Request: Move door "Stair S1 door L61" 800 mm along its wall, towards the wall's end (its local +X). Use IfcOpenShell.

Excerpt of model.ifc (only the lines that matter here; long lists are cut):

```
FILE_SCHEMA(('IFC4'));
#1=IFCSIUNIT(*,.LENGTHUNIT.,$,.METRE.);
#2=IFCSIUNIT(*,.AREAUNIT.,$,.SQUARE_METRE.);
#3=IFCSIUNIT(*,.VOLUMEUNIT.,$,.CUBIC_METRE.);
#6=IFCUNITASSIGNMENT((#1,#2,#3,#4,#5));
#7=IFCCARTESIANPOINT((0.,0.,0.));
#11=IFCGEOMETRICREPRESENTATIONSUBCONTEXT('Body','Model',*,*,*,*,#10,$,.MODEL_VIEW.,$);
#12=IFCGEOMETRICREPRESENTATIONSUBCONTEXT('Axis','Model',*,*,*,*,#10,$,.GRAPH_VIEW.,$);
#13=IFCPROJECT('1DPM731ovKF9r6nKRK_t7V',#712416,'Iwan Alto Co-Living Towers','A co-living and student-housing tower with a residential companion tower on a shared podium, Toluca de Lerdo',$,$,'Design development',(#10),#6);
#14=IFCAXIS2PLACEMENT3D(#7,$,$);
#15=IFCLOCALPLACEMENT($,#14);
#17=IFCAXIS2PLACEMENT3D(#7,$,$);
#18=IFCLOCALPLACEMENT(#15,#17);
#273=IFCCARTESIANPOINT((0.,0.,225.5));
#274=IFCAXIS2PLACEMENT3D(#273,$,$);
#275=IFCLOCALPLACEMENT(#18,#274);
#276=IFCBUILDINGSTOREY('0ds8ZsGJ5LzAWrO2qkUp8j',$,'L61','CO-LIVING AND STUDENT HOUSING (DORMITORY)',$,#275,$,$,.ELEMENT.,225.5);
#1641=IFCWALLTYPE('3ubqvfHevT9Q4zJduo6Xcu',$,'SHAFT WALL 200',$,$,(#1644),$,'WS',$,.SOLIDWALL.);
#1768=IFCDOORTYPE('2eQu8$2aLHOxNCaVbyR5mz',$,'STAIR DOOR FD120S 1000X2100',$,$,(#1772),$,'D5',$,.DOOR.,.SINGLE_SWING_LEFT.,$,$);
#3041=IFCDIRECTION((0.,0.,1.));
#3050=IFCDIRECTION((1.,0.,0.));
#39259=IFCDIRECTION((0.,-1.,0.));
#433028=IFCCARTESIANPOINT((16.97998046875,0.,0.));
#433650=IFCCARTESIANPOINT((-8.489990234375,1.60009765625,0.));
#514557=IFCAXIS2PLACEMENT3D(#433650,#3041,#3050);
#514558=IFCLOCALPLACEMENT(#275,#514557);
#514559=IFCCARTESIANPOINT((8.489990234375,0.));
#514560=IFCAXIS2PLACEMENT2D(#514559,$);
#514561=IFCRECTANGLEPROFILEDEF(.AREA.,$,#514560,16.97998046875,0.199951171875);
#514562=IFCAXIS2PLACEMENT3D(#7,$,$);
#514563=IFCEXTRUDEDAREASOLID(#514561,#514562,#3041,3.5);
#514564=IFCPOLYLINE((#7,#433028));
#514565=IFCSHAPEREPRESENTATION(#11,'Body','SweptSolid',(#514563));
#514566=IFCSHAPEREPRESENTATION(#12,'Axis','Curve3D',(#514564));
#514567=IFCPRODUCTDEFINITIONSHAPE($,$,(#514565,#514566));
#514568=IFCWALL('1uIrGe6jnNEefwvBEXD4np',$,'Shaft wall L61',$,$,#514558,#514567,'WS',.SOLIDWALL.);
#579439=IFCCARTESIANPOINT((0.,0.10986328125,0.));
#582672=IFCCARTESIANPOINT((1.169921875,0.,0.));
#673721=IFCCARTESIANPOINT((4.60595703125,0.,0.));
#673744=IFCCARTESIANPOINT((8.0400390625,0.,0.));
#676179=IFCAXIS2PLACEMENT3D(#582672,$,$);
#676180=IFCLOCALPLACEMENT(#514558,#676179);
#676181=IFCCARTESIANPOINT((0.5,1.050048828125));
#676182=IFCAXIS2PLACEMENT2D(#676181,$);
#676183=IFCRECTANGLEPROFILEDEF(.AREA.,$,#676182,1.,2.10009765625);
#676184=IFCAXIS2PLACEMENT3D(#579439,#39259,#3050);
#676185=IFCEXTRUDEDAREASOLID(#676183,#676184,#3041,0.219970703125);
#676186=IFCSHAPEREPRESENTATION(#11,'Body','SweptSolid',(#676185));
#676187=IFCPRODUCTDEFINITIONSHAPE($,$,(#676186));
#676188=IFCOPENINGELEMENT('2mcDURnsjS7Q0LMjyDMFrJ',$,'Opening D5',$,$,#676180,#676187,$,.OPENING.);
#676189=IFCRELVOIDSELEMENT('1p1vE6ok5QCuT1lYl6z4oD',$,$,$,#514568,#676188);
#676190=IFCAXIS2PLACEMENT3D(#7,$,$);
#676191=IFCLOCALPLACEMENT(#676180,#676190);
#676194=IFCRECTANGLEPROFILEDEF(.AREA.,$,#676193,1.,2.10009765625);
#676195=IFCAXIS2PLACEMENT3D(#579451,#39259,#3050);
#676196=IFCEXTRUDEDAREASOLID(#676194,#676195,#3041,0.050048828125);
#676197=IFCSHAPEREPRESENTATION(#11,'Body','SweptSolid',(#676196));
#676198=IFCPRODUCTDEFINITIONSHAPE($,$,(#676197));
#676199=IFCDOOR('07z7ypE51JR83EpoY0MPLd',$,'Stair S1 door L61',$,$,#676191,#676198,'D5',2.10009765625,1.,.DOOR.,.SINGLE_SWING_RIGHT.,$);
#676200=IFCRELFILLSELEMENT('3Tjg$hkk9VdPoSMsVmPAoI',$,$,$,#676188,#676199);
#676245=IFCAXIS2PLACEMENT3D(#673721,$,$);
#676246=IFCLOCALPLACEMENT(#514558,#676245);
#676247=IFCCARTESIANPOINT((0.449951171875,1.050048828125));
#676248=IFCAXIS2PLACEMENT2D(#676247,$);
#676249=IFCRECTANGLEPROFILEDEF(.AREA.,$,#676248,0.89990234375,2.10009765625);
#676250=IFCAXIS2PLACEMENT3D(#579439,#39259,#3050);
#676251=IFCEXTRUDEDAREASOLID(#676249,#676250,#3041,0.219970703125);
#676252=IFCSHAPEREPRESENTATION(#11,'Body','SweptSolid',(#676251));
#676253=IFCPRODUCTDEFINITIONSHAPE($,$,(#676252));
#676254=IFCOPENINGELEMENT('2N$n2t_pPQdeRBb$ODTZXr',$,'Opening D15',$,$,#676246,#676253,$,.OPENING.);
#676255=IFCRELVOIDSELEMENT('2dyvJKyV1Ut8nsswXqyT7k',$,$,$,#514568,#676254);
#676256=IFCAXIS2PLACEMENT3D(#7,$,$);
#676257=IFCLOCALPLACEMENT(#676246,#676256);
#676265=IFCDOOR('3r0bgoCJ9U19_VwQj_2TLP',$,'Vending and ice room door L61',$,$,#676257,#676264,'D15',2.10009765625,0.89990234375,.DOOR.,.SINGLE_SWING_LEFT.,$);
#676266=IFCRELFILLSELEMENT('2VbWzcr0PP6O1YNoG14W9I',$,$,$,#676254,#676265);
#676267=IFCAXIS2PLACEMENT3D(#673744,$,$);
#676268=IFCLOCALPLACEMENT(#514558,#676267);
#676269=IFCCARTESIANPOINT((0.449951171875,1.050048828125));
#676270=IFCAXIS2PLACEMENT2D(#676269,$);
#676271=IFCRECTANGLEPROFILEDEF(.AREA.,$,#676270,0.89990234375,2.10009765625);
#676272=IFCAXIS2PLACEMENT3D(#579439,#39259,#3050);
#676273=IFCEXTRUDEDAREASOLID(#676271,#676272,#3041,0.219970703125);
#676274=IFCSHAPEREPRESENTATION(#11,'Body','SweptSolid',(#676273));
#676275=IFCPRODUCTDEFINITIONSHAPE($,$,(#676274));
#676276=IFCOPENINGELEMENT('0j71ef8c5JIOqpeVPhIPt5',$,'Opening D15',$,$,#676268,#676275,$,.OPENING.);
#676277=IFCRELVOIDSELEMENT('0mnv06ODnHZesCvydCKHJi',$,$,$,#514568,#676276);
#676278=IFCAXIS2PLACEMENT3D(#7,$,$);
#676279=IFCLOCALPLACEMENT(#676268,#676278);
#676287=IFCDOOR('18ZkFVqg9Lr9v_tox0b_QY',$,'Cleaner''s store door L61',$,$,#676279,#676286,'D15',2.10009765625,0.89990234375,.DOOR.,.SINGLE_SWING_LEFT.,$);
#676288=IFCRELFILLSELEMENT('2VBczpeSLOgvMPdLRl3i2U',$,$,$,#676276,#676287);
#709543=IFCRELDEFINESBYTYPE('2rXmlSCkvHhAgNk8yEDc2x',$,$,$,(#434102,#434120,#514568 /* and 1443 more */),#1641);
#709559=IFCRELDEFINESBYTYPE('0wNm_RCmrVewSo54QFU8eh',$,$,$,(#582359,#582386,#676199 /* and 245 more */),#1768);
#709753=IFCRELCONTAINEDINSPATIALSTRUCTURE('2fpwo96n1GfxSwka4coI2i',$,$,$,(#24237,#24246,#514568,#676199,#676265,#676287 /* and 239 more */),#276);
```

```python
import ifcopenshell
import ifcopenshell.api.geometry
import ifcopenshell.util.placement

model = ifcopenshell.open("model.ifc")

door = model.by_id(676199)
opening = door.FillsVoids[0].RelatingOpeningElement
wall = opening.VoidsElements[0].RelatingBuildingElement

wall_matrix = ifcopenshell.util.placement.get_local_placement(wall.ObjectPlacement)
shift = wall_matrix[:3, 0] * 0.8
before = ifcopenshell.util.placement.get_local_placement(door.ObjectPlacement)[:3, 3].copy()

# The door is placed relative to its opening, so it follows when the opening moves.
matrix = ifcopenshell.util.placement.get_local_placement(opening.ObjectPlacement)
matrix[:3, 3] += shift
ifcopenshell.api.geometry.edit_object_placement(
    model, product=opening, matrix=matrix, is_si=False, should_transform_children=True
)

after = ifcopenshell.util.placement.get_local_placement(door.ObjectPlacement)[:3, 3]
print("door moved by", (after - before).round(3) + 0.0)

model.write("model_v2.ifc")
```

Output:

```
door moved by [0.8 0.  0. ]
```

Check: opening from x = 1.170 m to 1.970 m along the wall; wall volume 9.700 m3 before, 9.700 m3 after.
